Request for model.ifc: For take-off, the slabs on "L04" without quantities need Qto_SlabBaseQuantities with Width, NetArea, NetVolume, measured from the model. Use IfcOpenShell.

First a look at what the model holds.

```python
import ifcopenshell
import ifcopenshell.util.element
import ifcopenshell.util.unit

model = ifcopenshell.open("model.ifc")
print(model.schema)
for unit_type in ("LENGTHUNIT", "AREAUNIT", "VOLUMEUNIT"):
    print(unit_type, ifcopenshell.util.unit.calculate_unit_scale(model, unit_type))
storey = next(s for s in model.by_type("IfcBuildingStorey") if s.Name == "L04")
slabs = [e for e in ifcopenshell.util.element.get_decomposition(storey) if e.is_a("IfcSlab")]
for e in sorted(slabs, key=lambda e: e.id()):
    print(e.id(), e.is_a(), e.Name, list(ifcopenshell.util.element.get_psets(e, qtos_only=True)), sep=" | ")
```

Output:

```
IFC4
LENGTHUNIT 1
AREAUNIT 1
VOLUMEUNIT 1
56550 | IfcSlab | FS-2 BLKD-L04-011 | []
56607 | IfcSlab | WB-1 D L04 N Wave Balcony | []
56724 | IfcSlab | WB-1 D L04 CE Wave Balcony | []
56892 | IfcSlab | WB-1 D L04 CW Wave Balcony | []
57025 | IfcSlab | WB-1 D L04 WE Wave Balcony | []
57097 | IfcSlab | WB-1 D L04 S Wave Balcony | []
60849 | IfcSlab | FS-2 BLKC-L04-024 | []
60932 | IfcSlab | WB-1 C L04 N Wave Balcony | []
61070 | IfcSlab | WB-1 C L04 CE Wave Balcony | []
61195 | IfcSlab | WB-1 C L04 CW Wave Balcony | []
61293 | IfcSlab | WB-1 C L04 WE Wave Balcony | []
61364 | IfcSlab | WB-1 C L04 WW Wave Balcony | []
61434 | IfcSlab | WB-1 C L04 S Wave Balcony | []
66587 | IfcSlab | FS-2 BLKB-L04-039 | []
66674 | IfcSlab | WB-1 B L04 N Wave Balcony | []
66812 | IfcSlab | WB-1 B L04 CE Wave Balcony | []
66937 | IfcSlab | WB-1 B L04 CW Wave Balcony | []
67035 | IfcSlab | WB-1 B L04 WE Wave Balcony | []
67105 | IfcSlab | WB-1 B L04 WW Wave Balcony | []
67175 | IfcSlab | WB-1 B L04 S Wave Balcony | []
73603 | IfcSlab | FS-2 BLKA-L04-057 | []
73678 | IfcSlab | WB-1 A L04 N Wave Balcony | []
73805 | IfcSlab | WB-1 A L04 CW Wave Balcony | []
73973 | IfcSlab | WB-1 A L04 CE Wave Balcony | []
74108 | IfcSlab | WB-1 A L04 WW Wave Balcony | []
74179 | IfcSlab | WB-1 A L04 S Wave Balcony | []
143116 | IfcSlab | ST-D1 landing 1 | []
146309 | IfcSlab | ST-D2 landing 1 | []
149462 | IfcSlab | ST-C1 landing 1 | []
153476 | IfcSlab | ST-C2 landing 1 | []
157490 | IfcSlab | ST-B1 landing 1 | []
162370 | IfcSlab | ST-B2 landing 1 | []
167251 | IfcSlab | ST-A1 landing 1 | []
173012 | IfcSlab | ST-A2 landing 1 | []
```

```python
import ifcopenshell
import ifcopenshell.api.pset
import ifcopenshell.geom
import ifcopenshell.util.element
import ifcopenshell.util.shape
import ifcopenshell.util.unit

model = ifcopenshell.open("model.ifc")
unit_scale = ifcopenshell.util.unit.calculate_unit_scale(model)
area_scale = ifcopenshell.util.unit.calculate_unit_scale(model, "AREAUNIT")
volume_scale = ifcopenshell.util.unit.calculate_unit_scale(model, "VOLUMEUNIT")
settings = ifcopenshell.geom.settings()

storey = next(s for s in model.by_type("IfcBuildingStorey") if s.Name == "L04")
slabs = [e for e in ifcopenshell.util.element.get_decomposition(storey) if e.is_a("IfcSlab")]

for e in sorted(slabs, key=lambda e: e.id()):
    if ifcopenshell.util.element.get_psets(e, qtos_only=True, should_inherit=False):
        continue
    # Geometry comes back in metres, in the element's own axes.
    shape = ifcopenshell.geom.create_shape(settings, e)
    values = {
        "Width": ifcopenshell.util.shape.get_z(shape.geometry) / unit_scale,
        "NetArea": ifcopenshell.util.shape.get_footprint_area(shape.geometry) / area_scale,
        "NetVolume": ifcopenshell.util.shape.get_volume(shape.geometry) / volume_scale,
    }
    qto = ifcopenshell.api.pset.add_qto(model, product=e, name="Qto_SlabBaseQuantities")
    ifcopenshell.api.pset.edit_qto(model, qto=qto, properties=values)
    print(e.id(), {k: round(v, 3) for k, v in values.items()})

model.write("model_updated.ifc")
```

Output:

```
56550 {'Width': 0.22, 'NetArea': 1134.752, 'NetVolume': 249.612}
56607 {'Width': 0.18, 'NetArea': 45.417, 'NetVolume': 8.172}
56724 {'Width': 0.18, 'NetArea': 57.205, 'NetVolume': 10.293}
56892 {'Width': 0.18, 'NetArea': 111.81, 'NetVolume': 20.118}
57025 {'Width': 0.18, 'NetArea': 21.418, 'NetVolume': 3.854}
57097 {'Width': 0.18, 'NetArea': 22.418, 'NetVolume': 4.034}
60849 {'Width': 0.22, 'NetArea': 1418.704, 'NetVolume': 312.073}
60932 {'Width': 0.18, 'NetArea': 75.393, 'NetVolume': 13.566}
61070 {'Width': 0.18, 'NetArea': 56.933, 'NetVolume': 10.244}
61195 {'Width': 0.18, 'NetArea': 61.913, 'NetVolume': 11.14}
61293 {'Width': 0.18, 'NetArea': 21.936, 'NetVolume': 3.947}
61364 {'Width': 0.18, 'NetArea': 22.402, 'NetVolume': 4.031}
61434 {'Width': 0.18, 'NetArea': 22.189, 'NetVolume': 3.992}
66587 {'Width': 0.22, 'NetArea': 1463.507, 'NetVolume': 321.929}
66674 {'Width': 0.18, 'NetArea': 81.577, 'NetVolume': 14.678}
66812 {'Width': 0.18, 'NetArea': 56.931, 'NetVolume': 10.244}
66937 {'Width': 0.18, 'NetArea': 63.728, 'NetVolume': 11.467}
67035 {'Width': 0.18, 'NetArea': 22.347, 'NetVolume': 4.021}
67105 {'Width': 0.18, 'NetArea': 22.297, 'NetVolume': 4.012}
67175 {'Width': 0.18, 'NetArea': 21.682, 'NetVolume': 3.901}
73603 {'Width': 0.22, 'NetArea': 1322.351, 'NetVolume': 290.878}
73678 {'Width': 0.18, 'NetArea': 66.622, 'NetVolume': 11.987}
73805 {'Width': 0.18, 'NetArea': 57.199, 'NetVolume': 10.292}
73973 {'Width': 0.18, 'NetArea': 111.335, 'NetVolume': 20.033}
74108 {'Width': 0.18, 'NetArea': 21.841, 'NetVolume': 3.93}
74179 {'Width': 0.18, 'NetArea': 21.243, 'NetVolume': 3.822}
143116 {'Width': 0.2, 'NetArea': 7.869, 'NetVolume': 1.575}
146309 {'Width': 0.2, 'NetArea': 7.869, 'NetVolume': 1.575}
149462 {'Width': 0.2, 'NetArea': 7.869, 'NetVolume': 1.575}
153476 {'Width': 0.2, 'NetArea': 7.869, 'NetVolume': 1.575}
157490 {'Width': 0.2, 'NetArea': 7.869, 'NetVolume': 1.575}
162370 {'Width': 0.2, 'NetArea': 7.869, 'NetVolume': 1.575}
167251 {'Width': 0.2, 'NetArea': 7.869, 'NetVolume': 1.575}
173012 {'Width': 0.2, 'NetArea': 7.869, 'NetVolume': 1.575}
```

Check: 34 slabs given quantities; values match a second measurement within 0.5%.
